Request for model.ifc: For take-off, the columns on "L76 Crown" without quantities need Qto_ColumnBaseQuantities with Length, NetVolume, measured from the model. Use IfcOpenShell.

First a look at what the model holds.

```python
import ifcopenshell
import ifcopenshell.util.element
import ifcopenshell.util.unit

model = ifcopenshell.open("model.ifc")
print(model.schema)
for unit_type in ("LENGTHUNIT", "AREAUNIT", "VOLUMEUNIT"):
    print(unit_type, ifcopenshell.util.unit.calculate_unit_scale(model, unit_type))
storey = next(s for s in model.by_type("IfcBuildingStorey") if s.Name == "L76 Crown")
columns = [e for e in ifcopenshell.util.element.get_decomposition(storey) if e.is_a("IfcColumn")]
for e in sorted(columns, key=lambda e: e.id()):
    print(e.id(), e.is_a(), e.Name, list(ifcopenshell.util.element.get_psets(e, qtos_only=True)), sep=" | ")
```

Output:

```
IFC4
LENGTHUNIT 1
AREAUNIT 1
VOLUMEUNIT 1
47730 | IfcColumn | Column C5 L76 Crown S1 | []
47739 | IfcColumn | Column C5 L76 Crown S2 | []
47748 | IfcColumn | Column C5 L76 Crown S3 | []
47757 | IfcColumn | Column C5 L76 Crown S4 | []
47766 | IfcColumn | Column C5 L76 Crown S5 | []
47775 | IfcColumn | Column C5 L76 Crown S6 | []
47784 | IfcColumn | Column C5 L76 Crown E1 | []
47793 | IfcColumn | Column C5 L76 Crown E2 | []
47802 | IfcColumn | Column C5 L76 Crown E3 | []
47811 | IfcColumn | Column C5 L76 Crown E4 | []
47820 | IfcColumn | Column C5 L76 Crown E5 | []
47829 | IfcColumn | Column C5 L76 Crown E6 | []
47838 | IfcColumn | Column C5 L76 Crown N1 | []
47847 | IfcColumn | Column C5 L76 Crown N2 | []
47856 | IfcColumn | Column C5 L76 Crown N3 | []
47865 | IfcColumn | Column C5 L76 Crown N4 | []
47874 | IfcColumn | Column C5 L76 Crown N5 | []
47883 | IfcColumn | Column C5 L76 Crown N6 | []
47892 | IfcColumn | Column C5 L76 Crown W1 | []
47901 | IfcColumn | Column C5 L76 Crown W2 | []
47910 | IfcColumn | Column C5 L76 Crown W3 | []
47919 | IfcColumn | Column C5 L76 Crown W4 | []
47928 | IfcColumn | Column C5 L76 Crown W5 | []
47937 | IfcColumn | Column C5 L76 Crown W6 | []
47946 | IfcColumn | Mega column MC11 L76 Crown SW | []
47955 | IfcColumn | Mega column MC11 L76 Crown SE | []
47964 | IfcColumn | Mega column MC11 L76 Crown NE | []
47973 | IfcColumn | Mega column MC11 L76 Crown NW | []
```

```python
import ifcopenshell
import ifcopenshell.api.pset
import ifcopenshell.geom
import ifcopenshell.util.element
import ifcopenshell.util.shape
import ifcopenshell.util.unit

model = ifcopenshell.open("model.ifc")
unit_scale = ifcopenshell.util.unit.calculate_unit_scale(model)
volume_scale = ifcopenshell.util.unit.calculate_unit_scale(model, "VOLUMEUNIT")
settings = ifcopenshell.geom.settings()

storey = next(s for s in model.by_type("IfcBuildingStorey") if s.Name == "L76 Crown")
columns = [e for e in ifcopenshell.util.element.get_decomposition(storey) if e.is_a("IfcColumn")]

for e in sorted(columns, key=lambda e: e.id()):
    if ifcopenshell.util.element.get_psets(e, qtos_only=True, should_inherit=False):
        continue
    # Geometry comes back in metres, in the element's own axes.
    shape = ifcopenshell.geom.create_shape(settings, e)
    values = {
        "Length": ifcopenshell.util.shape.get_z(shape.geometry) / unit_scale,
        "NetVolume": ifcopenshell.util.shape.get_volume(shape.geometry) / volume_scale,
    }
    qto = ifcopenshell.api.pset.add_qto(model, product=e, name="Qto_ColumnBaseQuantities")
    ifcopenshell.api.pset.edit_qto(model, qto=qto, properties=values)
    print(e.id(), {k: round(v, 3) for k, v in values.items()})

model.write("model-out.ifc")
```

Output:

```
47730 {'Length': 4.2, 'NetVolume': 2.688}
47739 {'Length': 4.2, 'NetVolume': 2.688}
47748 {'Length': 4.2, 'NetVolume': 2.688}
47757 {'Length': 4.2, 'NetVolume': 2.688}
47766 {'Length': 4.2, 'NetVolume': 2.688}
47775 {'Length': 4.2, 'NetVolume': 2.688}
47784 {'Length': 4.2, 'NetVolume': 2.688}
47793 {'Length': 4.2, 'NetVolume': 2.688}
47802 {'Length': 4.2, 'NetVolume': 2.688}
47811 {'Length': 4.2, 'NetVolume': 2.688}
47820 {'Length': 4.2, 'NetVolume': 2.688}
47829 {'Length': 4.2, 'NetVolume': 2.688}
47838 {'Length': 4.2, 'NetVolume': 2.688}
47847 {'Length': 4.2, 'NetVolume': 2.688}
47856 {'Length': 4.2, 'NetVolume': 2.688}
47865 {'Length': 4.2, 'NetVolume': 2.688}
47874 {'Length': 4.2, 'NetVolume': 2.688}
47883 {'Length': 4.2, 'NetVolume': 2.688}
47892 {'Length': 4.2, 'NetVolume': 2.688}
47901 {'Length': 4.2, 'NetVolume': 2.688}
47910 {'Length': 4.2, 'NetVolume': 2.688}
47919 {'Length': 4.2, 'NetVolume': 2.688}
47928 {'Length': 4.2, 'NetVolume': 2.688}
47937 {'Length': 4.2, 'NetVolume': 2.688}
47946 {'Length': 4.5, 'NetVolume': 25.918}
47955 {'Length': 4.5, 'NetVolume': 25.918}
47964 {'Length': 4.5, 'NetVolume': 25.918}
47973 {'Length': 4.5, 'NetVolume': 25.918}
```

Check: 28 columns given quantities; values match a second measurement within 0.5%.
